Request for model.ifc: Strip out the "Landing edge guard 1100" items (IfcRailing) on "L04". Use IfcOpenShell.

First a look at what the model holds.

```python
import ifcopenshell
import ifcopenshell.util.element

model = ifcopenshell.open("model.ifc")
print(model.schema)
storey = next(s for s in model.by_type("IfcBuildingStorey") if s.Name == "L04")
railings = [e for e in ifcopenshell.util.element.get_decomposition(storey) if e.is_a("IfcRailing")]
seen = {}
for e in railings:
    element_type = ifcopenshell.util.element.get_type(e)
    name = element_type.Name if element_type not in (None, e) else None
    seen[name] = seen.get(name, 0) + 1
for name, count in sorted(seen.items(), key=str):
    print(count, "x", name)
```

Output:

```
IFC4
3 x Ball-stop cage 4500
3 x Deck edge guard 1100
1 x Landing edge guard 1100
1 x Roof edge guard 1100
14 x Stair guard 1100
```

```python
import ifcopenshell
import ifcopenshell.api.root
import ifcopenshell.util.element

model = ifcopenshell.open("model.ifc")

storey = next(s for s in model.by_type("IfcBuildingStorey") if s.Name == "L04")
railings = [e for e in ifcopenshell.util.element.get_decomposition(storey) if e.is_a("IfcRailing")]
targets = [e for e in railings if (t := ifcopenshell.util.element.get_type(e)) not in (None, e) and t.Name == "Landing edge guard 1100"]

for e in targets:
    ifcopenshell.api.root.remove_product(model, product=e)
print(len(targets), "removed")

model.write("model_edited.ifc")
```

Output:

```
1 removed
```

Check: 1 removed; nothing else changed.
